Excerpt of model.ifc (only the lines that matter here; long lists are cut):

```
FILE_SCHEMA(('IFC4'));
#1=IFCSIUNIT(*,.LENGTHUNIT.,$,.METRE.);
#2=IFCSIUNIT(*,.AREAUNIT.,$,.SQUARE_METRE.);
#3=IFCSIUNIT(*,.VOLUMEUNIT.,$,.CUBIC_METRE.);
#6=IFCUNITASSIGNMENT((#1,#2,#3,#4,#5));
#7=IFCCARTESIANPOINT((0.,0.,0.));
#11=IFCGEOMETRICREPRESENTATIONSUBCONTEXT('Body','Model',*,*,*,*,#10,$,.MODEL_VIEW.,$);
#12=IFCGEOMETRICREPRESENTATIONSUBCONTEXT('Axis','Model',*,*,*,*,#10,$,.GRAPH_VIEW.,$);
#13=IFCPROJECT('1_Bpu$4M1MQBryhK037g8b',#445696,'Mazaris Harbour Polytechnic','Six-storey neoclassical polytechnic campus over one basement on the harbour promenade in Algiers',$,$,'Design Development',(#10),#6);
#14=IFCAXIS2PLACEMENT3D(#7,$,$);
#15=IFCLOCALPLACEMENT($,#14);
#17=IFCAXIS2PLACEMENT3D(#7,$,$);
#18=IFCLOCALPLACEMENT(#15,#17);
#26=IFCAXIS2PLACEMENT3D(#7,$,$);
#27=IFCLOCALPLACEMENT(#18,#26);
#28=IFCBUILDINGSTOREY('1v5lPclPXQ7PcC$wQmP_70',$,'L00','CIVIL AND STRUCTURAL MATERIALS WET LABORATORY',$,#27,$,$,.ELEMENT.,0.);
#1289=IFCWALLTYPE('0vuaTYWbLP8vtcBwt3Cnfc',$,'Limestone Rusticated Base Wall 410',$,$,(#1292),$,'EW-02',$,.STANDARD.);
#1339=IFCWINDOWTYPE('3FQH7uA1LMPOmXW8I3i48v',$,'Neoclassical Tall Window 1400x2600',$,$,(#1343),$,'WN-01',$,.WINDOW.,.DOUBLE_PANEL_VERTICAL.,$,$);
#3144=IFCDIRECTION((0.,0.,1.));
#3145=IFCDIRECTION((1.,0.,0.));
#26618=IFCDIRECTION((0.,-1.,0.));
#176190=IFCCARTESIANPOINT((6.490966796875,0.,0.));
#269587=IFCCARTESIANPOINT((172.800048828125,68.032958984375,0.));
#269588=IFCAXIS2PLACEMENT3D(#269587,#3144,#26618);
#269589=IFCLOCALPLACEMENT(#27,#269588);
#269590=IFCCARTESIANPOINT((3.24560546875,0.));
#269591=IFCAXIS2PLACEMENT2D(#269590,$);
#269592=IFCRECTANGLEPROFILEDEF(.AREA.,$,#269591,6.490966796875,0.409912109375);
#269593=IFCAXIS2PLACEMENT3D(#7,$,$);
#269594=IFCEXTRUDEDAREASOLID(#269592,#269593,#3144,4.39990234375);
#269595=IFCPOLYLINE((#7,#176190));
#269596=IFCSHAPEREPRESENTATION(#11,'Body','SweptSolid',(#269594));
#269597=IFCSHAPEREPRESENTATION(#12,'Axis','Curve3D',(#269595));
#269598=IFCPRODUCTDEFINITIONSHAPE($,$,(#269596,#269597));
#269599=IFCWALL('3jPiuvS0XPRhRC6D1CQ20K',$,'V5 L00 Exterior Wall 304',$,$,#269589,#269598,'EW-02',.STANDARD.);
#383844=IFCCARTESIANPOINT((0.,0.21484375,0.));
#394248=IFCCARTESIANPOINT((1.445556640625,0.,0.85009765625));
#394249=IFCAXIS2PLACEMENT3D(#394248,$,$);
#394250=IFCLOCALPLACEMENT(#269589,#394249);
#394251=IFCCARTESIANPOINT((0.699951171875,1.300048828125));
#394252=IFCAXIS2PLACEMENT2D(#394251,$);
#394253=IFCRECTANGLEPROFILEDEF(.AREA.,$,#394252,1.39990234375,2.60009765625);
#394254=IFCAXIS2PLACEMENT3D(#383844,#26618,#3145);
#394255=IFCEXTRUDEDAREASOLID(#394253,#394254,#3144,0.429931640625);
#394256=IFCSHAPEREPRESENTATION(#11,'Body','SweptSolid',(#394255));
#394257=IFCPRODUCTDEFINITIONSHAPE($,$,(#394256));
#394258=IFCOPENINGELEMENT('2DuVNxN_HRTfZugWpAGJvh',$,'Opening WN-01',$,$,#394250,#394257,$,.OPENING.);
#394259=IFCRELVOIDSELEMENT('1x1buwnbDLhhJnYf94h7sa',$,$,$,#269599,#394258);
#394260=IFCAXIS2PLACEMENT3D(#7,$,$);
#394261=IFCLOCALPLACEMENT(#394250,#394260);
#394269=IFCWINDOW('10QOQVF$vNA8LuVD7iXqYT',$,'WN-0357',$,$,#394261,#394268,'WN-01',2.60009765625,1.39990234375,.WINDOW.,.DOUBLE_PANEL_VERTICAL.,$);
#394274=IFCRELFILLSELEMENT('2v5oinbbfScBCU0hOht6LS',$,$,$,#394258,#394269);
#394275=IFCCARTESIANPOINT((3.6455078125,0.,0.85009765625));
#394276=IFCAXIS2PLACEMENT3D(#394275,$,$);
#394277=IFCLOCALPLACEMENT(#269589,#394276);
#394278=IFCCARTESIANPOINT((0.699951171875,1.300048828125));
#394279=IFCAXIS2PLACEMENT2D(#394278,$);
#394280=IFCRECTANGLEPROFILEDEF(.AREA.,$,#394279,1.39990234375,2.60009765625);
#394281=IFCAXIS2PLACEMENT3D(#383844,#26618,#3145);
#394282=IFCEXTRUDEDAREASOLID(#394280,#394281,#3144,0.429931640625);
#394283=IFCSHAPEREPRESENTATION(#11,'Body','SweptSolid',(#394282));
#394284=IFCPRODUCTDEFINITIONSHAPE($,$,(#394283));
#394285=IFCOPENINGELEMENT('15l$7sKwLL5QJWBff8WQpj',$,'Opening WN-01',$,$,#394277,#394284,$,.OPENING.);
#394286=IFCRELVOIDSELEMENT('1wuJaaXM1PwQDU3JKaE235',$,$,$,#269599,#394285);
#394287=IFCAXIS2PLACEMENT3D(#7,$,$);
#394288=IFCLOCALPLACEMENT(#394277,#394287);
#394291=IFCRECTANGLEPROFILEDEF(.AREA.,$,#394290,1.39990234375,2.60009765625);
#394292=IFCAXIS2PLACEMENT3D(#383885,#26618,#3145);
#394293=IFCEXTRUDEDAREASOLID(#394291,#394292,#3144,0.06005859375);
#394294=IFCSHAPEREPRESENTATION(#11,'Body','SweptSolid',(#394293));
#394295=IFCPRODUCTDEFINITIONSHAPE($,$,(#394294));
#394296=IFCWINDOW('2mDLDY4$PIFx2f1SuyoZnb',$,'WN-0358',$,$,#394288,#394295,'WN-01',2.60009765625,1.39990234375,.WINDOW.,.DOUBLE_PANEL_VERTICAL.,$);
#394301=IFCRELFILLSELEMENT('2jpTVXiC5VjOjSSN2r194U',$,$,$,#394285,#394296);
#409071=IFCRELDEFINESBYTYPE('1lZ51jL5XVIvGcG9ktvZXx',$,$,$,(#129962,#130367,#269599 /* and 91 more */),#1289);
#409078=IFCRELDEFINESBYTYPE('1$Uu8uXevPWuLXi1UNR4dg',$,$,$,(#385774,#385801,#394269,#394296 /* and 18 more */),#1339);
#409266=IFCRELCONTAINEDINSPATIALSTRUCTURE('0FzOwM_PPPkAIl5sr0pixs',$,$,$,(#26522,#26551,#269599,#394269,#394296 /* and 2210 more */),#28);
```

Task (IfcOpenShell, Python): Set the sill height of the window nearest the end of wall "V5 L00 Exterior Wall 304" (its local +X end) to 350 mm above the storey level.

```python
import numpy as np
import ifcopenshell
import ifcopenshell.api.geometry
import ifcopenshell.geom
import ifcopenshell.util.element
import ifcopenshell.util.placement
import ifcopenshell.util.shape
import ifcopenshell.util.unit

model = ifcopenshell.open("model.ifc")
unit_scale = ifcopenshell.util.unit.calculate_unit_scale(model)

window = model.by_guid("2mDLDY4$PIFx2f1SuyoZnb")
opening = window.FillsVoids[0].RelatingOpeningElement
storey = ifcopenshell.util.element.get_container(window, ifc_class="IfcBuildingStorey")
level = ifcopenshell.util.placement.get_local_placement(storey.ObjectPlacement)[2, 3]

# The opening's origin need not be at the sill, so measure its lowest point.
shape = ifcopenshell.geom.create_shape(ifcopenshell.geom.settings(), opening)
bottom = ifcopenshell.util.shape.get_shape_bottom_elevation(shape, shape.geometry) / unit_scale
dz = level + 0.35 - bottom

shift = np.array([0.0, 0.0, dz])
# The window is placed relative to its opening, so it follows when the opening moves.
matrix = ifcopenshell.util.placement.get_local_placement(opening.ObjectPlacement)
matrix[:3, 3] += shift
ifcopenshell.api.geometry.edit_object_placement(
    model, product=opening, matrix=matrix, is_si=False, should_transform_children=True
)

print(f"moved by {dz * unit_scale:+.3f} m")

model.write("model_edited.ifc")
```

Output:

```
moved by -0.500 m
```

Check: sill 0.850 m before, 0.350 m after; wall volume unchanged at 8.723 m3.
